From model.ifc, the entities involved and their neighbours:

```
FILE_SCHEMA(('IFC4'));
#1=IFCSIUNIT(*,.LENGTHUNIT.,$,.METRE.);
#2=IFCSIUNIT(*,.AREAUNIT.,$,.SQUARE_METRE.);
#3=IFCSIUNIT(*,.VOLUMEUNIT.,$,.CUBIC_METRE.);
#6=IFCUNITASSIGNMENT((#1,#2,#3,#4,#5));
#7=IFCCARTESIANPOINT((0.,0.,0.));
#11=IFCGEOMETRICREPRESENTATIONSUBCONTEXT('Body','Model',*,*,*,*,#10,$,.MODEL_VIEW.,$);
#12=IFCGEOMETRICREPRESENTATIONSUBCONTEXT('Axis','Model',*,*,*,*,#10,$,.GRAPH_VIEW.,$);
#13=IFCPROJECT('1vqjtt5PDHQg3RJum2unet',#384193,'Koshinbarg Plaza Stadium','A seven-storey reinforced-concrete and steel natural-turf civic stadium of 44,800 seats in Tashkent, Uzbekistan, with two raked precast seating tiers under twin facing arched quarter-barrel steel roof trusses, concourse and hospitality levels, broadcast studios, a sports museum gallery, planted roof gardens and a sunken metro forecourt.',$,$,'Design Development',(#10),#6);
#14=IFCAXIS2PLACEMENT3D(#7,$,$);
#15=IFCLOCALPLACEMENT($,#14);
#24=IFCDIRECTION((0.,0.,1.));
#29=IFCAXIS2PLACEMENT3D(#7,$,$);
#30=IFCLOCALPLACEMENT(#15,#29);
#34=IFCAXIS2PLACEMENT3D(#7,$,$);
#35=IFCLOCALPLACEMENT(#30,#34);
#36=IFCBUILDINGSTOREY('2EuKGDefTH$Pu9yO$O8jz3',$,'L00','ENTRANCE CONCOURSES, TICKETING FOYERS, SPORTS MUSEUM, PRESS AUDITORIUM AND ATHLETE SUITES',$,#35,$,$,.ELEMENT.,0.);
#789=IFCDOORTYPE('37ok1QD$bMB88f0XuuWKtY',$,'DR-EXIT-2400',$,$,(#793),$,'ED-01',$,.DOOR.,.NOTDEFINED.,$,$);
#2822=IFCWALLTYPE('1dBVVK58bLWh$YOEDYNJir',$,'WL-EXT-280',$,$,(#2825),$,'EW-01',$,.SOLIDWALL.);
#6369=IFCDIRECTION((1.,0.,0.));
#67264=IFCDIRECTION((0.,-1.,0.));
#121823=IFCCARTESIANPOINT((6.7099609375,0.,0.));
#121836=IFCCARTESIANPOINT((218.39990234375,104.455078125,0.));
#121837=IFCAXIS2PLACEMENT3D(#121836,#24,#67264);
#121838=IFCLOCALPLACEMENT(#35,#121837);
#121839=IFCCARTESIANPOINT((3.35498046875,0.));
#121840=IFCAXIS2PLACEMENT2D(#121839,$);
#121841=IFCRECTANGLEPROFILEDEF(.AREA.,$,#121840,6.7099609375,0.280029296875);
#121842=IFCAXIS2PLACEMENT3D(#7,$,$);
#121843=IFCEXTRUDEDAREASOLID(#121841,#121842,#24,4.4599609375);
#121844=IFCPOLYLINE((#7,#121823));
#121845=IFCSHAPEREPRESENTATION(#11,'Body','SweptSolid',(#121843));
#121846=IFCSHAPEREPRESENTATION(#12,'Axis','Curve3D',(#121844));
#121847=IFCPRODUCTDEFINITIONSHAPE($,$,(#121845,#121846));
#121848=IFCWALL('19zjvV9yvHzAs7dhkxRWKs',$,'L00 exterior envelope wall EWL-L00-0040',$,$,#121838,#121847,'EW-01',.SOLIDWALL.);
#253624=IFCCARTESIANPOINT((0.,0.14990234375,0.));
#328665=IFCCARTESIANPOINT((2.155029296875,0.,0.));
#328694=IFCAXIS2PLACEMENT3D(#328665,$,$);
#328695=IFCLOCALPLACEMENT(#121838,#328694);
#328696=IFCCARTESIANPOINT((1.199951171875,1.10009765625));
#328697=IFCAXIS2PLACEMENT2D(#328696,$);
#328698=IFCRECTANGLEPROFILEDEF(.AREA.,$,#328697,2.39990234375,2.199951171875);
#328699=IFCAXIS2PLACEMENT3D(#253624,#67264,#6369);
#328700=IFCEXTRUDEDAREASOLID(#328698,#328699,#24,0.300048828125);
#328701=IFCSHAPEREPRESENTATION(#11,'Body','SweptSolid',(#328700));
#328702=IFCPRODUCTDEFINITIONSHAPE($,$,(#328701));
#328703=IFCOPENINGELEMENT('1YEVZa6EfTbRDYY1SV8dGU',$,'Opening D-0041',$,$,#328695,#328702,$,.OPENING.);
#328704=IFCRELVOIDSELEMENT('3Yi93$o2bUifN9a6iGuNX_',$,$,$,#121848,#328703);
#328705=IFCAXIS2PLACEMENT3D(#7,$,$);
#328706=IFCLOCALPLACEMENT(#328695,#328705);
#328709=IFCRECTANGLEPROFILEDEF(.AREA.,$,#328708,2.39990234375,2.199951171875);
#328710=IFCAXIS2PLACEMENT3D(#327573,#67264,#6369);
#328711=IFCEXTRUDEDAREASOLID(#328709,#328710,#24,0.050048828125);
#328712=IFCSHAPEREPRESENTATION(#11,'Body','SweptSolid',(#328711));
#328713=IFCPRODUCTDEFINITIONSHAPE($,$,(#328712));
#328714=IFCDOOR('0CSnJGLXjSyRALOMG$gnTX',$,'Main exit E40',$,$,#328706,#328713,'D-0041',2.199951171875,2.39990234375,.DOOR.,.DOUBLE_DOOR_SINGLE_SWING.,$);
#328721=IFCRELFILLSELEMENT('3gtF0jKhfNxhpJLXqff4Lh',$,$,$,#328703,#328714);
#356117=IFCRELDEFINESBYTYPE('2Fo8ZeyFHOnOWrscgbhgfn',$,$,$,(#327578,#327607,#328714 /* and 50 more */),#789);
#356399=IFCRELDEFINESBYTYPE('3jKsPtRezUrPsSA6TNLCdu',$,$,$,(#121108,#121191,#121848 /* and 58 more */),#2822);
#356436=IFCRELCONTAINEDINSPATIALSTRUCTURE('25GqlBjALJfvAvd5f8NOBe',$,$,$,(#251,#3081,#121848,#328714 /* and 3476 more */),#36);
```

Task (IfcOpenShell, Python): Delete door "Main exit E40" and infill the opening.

```python
import ifcopenshell
import ifcopenshell.api.feature
import ifcopenshell.api.root
import ifcopenshell.geom
import ifcopenshell.util.shape

model = ifcopenshell.open("model.ifc")
settings = ifcopenshell.geom.settings()


def volume(element):
    """Net volume in cubic metres, openings subtracted."""
    shape = ifcopenshell.geom.create_shape(settings, element)
    return ifcopenshell.util.shape.get_volume(shape.geometry)


door = model.by_guid("0CSnJGLXjSyRALOMG$gnTX")
opening = door.FillsVoids[0].RelatingOpeningElement
wall = opening.VoidsElements[0].RelatingBuildingElement
before = volume(wall)

ifcopenshell.api.root.remove_product(model, product=door)
ifcopenshell.api.feature.remove_feature(model, feature=opening)

after = volume(wall)

print(f"wall volume {before:.3f} -> {after:.3f} m3")

model.write("model_edited.ifc")
```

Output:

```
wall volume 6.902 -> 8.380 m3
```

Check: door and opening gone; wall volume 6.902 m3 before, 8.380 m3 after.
